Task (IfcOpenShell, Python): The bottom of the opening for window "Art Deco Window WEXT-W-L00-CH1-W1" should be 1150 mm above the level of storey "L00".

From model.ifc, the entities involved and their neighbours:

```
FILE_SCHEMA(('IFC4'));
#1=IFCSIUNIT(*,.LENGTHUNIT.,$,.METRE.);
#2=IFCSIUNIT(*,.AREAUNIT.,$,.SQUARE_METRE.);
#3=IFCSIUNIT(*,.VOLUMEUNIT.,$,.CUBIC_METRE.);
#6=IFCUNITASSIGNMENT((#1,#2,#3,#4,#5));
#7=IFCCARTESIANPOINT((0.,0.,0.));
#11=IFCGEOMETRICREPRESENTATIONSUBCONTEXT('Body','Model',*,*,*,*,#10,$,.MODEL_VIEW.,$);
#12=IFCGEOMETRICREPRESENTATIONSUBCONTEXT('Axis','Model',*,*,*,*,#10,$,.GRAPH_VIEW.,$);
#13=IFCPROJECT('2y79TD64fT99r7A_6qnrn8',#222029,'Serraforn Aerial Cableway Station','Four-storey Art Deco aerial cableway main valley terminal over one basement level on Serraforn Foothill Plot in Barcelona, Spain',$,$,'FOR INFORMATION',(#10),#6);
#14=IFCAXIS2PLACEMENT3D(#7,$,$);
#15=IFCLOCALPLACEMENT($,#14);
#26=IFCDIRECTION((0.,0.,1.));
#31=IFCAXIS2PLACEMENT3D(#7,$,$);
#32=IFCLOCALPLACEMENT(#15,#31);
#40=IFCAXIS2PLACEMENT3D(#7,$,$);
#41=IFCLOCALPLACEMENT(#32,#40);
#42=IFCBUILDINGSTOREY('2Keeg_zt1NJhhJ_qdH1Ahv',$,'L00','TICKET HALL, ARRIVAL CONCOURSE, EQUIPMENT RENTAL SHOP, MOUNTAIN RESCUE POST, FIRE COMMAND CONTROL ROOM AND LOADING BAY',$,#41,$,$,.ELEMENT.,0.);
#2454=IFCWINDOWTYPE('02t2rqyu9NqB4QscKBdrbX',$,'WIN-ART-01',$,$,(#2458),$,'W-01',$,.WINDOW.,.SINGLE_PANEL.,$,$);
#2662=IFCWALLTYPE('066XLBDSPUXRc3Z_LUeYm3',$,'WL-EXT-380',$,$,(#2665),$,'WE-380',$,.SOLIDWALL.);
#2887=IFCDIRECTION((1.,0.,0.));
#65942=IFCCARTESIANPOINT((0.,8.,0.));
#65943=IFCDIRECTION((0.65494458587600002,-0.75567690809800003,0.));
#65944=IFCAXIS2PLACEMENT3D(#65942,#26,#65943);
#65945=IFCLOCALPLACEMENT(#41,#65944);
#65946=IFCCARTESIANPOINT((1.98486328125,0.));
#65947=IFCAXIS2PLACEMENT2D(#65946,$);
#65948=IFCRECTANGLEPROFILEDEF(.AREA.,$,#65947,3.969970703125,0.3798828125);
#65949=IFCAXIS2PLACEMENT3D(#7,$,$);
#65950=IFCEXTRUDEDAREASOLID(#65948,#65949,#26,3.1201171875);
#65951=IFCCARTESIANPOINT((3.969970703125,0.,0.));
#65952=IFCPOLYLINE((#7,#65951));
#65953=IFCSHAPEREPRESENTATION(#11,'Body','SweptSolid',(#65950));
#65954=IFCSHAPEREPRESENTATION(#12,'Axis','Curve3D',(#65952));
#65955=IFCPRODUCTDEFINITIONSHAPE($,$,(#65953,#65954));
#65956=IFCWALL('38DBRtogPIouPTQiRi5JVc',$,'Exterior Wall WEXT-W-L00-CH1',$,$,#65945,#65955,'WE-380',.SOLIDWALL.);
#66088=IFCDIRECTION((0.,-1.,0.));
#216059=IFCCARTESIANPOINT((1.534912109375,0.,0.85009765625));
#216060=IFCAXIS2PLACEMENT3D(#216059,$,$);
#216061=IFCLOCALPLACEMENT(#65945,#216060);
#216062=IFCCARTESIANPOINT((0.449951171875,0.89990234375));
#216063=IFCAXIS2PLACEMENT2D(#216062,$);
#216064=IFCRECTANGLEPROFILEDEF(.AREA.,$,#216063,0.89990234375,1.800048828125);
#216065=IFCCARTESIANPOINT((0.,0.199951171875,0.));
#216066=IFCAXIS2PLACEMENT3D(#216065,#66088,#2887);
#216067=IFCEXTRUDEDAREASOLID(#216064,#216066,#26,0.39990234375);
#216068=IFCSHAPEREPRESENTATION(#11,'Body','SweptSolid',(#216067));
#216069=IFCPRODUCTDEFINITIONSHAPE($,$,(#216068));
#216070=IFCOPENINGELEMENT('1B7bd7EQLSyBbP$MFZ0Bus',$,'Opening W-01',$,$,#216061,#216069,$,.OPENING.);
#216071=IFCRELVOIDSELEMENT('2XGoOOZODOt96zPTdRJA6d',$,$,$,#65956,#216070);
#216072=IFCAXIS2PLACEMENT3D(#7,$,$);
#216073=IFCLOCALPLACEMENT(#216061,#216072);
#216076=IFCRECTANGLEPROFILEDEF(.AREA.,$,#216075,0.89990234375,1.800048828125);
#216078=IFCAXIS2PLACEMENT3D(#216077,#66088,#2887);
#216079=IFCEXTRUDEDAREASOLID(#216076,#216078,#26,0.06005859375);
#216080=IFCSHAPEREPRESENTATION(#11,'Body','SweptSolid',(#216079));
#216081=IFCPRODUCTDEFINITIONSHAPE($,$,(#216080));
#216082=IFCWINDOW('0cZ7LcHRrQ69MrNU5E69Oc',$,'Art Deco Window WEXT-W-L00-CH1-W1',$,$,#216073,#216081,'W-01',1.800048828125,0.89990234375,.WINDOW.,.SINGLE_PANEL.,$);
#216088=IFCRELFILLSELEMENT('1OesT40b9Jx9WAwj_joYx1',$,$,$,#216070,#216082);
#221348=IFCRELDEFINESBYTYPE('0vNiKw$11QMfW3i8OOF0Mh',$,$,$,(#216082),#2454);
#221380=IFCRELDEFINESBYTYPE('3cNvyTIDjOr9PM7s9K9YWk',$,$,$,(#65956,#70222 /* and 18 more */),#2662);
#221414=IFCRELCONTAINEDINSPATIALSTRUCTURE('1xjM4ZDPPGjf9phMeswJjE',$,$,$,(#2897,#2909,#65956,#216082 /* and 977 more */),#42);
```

```python
import numpy as np
import ifcopenshell
import ifcopenshell.api.geometry
import ifcopenshell.geom
import ifcopenshell.util.element
import ifcopenshell.util.placement
import ifcopenshell.util.shape
import ifcopenshell.util.unit

model = ifcopenshell.open("model.ifc")
unit_scale = ifcopenshell.util.unit.calculate_unit_scale(model)

window = model.by_guid("0cZ7LcHRrQ69MrNU5E69Oc")
opening = window.FillsVoids[0].RelatingOpeningElement
storey = ifcopenshell.util.element.get_container(window, ifc_class="IfcBuildingStorey")
level = ifcopenshell.util.placement.get_local_placement(storey.ObjectPlacement)[2, 3]

# The opening's origin need not be at the sill, so measure its lowest point.
shape = ifcopenshell.geom.create_shape(ifcopenshell.geom.settings(), opening)
bottom = ifcopenshell.util.shape.get_shape_bottom_elevation(shape, shape.geometry) / unit_scale
dz = level + 1.15 / unit_scale - bottom

shift = np.array([0.0, 0.0, dz])
# The window is placed relative to its opening, so it follows when the opening moves.
matrix = ifcopenshell.util.placement.get_local_placement(opening.ObjectPlacement)
matrix[:3, 3] += shift
ifcopenshell.api.geometry.edit_object_placement(
    model, product=opening, matrix=matrix, is_si=False, should_transform_children=True
)

print(f"moved by {dz * unit_scale:+.3f} m")

model.write("model_updated.ifc")
```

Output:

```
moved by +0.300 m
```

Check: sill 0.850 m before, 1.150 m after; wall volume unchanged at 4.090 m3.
